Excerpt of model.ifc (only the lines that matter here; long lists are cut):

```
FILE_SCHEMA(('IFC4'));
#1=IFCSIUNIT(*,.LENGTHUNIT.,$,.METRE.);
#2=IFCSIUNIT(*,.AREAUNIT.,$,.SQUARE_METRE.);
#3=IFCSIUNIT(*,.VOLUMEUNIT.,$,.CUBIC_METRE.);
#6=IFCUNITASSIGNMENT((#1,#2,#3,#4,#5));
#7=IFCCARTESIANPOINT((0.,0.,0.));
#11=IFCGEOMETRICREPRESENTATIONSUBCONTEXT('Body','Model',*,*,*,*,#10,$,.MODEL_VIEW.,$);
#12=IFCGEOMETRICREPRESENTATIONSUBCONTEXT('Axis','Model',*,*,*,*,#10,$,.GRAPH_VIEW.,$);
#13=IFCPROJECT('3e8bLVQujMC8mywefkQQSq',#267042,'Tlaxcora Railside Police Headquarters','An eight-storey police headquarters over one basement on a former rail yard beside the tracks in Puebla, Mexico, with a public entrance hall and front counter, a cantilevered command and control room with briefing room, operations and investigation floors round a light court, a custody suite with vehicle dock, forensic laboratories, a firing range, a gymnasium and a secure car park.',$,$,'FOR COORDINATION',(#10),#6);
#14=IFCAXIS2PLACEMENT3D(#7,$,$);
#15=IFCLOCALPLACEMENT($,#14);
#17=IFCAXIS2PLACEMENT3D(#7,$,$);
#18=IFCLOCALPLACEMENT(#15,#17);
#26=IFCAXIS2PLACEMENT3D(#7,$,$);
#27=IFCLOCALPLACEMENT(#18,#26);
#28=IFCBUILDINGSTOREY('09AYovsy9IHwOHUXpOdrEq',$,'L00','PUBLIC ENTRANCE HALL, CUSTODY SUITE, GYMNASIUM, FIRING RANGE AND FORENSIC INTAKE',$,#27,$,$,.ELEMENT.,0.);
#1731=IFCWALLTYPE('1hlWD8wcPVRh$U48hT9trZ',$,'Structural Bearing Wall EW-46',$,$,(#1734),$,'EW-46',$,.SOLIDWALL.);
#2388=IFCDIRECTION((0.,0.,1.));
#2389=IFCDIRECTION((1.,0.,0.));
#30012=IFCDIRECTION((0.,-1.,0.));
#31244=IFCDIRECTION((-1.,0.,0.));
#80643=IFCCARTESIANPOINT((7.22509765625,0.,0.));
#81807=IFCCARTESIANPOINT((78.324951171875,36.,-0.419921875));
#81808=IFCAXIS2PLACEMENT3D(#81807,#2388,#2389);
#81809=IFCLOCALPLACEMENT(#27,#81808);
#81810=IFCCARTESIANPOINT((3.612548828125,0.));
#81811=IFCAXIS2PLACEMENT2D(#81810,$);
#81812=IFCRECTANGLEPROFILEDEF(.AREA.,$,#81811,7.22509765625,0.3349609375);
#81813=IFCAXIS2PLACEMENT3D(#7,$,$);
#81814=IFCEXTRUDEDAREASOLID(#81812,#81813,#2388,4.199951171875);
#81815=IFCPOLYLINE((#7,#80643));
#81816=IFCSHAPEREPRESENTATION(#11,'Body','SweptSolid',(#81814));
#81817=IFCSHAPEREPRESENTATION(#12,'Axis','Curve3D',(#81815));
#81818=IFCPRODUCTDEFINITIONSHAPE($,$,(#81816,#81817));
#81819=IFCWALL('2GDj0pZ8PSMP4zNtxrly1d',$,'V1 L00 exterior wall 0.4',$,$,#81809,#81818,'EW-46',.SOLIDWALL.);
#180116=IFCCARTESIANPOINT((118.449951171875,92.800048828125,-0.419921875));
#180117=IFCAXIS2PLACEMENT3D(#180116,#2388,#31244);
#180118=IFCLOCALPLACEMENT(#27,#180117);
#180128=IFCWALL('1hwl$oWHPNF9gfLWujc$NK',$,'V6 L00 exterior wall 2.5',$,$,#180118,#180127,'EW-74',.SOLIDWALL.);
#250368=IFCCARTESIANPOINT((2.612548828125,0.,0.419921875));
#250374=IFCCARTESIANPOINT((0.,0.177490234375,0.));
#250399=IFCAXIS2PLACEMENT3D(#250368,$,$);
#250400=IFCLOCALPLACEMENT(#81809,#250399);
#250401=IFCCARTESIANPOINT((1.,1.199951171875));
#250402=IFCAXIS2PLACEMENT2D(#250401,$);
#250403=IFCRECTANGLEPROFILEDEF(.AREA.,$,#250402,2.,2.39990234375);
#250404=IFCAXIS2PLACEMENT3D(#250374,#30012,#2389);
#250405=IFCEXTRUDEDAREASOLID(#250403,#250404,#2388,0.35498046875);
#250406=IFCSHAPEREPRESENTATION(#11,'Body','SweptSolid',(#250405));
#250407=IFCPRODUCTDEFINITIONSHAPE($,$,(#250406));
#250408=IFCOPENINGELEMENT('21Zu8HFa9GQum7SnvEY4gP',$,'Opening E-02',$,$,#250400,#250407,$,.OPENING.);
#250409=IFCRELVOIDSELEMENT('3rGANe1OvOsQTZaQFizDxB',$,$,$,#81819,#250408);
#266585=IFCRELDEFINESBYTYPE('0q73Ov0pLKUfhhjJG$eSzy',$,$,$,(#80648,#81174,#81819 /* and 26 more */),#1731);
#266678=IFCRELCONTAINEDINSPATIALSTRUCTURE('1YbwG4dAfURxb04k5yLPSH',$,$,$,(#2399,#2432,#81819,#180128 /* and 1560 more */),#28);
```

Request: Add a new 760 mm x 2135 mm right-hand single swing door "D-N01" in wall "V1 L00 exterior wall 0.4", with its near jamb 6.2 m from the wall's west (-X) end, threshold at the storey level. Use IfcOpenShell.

```python
import numpy as np
import ifcopenshell
import ifcopenshell.api.feature
import ifcopenshell.api.geometry
import ifcopenshell.api.root
import ifcopenshell.api.spatial
import ifcopenshell.geom
import ifcopenshell.util.element
import ifcopenshell.util.placement
import ifcopenshell.util.representation
import ifcopenshell.util.shape
import ifcopenshell.util.unit

model = ifcopenshell.open("model.ifc")
unit_scale = ifcopenshell.util.unit.calculate_unit_scale(model)
settings = ifcopenshell.geom.settings()


def volume(element):
    """Net volume in cubic metres, openings subtracted."""
    shape = ifcopenshell.geom.create_shape(settings, element)
    return ifcopenshell.util.shape.get_volume(shape.geometry)


wall = model.by_id(81819)
storey = ifcopenshell.util.element.get_container(wall, ifc_class="IfcBuildingStorey")
context = ifcopenshell.util.representation.get_context(model, "Model", "Body", "MODEL_VIEW")
before = volume(wall)

width, height, from_end, sill = 0.76, 2.135, 6.2, 0.0  # metres

# The wall runs along its own X axis, and the end named is its -X end.
wall_shape = ifcopenshell.geom.create_shape(settings, wall)
x, y, z = ifcopenshell.util.shape.get_vertices(wall_shape.geometry).T
start = x.min() + from_end
face, thickness = float(y.min()), float(y.max() - y.min())
wall_matrix = ifcopenshell.util.placement.get_local_placement(wall.ObjectPlacement)
level = ifcopenshell.util.placement.get_local_placement(storey.ObjectPlacement)[2, 3]


def in_wall(x, y):
    """Placement at x, y metres in the wall's axes, at sill height."""
    matrix = wall_matrix.copy()
    matrix[:, 3] = wall_matrix @ np.array([x / unit_scale, y / unit_scale, 0.0, 1.0])
    matrix[2, 3] = level + sill / unit_scale
    return matrix


# Opening: a box that overshoots both wall faces by 50 mm.
opening = ifcopenshell.api.root.create_entity(model, ifc_class="IfcOpeningElement", predefined_type="OPENING")
box = ifcopenshell.api.geometry.add_wall_representation(
    model, context=context, length=width, height=height, thickness=thickness + 0.1
)
ifcopenshell.api.geometry.assign_representation(model, product=opening, representation=box)
ifcopenshell.api.geometry.edit_object_placement(model, product=opening, matrix=in_wall(start, face - 0.05), is_si=False)
ifcopenshell.api.feature.add_feature(model, feature=opening, element=wall)

door = ifcopenshell.api.root.create_entity(model, ifc_class="IfcDoor", name="D-N01", predefined_type="DOOR")
door.OverallWidth, door.OverallHeight = width / unit_scale, height / unit_scale
door.OperationType = "SINGLE_SWING_RIGHT"
body = ifcopenshell.api.geometry.add_door_representation(
    model,
    context=context,
    overall_width=door.OverallWidth,
    overall_height=door.OverallHeight,
    operation_type="SINGLE_SWING_RIGHT",
    lining_properties={"LiningDepth": thickness / unit_scale, "ThresholdDepth": thickness / unit_scale},
)
ifcopenshell.api.geometry.assign_representation(model, product=door, representation=body)
ifcopenshell.api.spatial.assign_container(model, products=[door], relating_structure=storey)
ifcopenshell.api.feature.add_filling(model, opening=opening, element=door)

# The lining spans the wall, so the door starts at the wall face.
ifcopenshell.api.geometry.edit_object_placement(model, product=door, matrix=in_wall(start, face), is_si=False)

after = volume(wall)

print(f"wall volume {before:.3f} -> {after:.3f} m3")

model.write("model_updated.ifc")
```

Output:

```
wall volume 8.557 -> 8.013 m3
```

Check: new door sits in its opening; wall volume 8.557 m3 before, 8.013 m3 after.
